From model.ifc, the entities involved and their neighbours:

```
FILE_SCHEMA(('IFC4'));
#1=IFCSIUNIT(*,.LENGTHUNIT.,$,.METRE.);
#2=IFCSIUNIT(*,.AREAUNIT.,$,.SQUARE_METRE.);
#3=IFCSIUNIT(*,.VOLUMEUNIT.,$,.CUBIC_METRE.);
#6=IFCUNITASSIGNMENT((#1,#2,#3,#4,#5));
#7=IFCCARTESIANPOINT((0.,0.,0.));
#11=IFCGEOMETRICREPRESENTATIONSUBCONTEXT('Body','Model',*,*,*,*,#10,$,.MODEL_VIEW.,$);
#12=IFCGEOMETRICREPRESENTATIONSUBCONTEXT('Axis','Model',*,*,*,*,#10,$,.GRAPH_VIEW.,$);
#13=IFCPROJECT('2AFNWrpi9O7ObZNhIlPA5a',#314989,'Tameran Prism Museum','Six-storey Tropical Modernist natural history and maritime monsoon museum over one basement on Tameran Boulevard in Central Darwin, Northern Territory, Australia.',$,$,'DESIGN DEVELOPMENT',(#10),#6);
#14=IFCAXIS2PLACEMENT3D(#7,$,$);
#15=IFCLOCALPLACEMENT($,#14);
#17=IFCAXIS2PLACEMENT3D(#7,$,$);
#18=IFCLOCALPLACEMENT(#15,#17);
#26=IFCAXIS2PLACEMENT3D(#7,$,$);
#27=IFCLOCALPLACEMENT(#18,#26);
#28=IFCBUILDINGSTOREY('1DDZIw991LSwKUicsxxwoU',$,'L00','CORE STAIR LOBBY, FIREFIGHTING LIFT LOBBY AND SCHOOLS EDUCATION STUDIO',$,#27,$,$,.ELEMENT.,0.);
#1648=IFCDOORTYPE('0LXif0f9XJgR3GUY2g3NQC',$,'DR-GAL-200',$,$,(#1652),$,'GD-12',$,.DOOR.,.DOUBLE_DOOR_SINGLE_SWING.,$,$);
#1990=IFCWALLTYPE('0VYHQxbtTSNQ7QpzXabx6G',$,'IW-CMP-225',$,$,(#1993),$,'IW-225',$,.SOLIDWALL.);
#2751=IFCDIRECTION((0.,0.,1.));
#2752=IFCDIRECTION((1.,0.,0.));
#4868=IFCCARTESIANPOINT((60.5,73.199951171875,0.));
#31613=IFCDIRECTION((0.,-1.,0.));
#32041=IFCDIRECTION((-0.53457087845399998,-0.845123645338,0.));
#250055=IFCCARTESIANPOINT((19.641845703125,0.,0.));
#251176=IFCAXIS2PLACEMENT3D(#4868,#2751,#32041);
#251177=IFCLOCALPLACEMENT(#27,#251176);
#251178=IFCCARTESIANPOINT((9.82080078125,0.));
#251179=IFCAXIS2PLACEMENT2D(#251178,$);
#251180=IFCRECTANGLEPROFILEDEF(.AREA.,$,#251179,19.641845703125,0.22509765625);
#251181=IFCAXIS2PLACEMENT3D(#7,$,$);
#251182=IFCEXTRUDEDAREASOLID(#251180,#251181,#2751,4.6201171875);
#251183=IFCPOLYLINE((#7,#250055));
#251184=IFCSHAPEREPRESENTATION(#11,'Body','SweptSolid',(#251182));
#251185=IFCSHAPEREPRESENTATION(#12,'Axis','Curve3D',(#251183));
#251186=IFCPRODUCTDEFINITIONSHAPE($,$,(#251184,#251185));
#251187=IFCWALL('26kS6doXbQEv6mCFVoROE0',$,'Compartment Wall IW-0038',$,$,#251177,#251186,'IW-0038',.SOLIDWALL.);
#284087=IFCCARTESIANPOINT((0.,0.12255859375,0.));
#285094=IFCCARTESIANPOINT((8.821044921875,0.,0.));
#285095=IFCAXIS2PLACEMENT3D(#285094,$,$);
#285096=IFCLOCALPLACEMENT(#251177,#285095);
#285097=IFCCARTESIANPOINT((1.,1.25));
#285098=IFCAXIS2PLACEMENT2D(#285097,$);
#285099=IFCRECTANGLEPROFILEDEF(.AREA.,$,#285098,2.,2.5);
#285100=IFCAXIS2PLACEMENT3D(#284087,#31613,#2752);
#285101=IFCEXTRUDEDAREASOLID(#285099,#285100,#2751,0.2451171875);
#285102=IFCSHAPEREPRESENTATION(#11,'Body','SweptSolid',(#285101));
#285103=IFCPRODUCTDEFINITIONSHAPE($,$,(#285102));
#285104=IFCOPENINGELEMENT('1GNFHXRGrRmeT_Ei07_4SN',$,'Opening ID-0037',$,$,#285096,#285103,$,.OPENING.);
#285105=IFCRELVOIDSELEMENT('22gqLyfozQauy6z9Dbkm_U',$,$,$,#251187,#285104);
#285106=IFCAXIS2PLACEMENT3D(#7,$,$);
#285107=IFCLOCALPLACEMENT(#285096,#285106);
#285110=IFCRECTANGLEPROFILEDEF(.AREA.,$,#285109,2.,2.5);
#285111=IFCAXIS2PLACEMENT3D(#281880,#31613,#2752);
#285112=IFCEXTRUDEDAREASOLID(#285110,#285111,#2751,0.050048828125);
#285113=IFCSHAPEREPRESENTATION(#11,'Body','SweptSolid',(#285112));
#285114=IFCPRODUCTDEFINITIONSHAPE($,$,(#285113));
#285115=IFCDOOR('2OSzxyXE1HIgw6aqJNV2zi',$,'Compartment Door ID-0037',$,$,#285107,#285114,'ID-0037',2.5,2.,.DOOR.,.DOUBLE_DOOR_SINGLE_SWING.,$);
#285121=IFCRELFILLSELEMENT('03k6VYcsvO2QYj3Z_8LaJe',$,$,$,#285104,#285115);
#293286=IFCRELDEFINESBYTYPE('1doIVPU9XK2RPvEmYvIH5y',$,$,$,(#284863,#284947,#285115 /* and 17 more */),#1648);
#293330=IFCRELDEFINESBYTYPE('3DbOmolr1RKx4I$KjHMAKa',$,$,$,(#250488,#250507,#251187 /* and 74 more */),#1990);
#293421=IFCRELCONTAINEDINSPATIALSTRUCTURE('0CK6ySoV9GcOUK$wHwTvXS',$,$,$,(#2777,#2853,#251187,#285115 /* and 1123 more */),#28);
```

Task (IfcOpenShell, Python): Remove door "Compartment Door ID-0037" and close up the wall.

```python
import ifcopenshell
import ifcopenshell.api.feature
import ifcopenshell.api.root
import ifcopenshell.geom
import ifcopenshell.util.shape

model = ifcopenshell.open("model.ifc")
settings = ifcopenshell.geom.settings()


def volume(element):
    """Net volume in cubic metres, openings subtracted."""
    shape = ifcopenshell.geom.create_shape(settings, element)
    return ifcopenshell.util.shape.get_volume(shape.geometry)


door = model.by_id(285115)
opening = door.FillsVoids[0].RelatingOpeningElement
wall = opening.VoidsElements[0].RelatingBuildingElement
before = volume(wall)

ifcopenshell.api.root.remove_product(model, product=door)
ifcopenshell.api.feature.remove_feature(model, feature=opening)

after = volume(wall)

print(f"wall volume {before:.3f} -> {after:.3f} m3")

model.write("model-out.ifc")
```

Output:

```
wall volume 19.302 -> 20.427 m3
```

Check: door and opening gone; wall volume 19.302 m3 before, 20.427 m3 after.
